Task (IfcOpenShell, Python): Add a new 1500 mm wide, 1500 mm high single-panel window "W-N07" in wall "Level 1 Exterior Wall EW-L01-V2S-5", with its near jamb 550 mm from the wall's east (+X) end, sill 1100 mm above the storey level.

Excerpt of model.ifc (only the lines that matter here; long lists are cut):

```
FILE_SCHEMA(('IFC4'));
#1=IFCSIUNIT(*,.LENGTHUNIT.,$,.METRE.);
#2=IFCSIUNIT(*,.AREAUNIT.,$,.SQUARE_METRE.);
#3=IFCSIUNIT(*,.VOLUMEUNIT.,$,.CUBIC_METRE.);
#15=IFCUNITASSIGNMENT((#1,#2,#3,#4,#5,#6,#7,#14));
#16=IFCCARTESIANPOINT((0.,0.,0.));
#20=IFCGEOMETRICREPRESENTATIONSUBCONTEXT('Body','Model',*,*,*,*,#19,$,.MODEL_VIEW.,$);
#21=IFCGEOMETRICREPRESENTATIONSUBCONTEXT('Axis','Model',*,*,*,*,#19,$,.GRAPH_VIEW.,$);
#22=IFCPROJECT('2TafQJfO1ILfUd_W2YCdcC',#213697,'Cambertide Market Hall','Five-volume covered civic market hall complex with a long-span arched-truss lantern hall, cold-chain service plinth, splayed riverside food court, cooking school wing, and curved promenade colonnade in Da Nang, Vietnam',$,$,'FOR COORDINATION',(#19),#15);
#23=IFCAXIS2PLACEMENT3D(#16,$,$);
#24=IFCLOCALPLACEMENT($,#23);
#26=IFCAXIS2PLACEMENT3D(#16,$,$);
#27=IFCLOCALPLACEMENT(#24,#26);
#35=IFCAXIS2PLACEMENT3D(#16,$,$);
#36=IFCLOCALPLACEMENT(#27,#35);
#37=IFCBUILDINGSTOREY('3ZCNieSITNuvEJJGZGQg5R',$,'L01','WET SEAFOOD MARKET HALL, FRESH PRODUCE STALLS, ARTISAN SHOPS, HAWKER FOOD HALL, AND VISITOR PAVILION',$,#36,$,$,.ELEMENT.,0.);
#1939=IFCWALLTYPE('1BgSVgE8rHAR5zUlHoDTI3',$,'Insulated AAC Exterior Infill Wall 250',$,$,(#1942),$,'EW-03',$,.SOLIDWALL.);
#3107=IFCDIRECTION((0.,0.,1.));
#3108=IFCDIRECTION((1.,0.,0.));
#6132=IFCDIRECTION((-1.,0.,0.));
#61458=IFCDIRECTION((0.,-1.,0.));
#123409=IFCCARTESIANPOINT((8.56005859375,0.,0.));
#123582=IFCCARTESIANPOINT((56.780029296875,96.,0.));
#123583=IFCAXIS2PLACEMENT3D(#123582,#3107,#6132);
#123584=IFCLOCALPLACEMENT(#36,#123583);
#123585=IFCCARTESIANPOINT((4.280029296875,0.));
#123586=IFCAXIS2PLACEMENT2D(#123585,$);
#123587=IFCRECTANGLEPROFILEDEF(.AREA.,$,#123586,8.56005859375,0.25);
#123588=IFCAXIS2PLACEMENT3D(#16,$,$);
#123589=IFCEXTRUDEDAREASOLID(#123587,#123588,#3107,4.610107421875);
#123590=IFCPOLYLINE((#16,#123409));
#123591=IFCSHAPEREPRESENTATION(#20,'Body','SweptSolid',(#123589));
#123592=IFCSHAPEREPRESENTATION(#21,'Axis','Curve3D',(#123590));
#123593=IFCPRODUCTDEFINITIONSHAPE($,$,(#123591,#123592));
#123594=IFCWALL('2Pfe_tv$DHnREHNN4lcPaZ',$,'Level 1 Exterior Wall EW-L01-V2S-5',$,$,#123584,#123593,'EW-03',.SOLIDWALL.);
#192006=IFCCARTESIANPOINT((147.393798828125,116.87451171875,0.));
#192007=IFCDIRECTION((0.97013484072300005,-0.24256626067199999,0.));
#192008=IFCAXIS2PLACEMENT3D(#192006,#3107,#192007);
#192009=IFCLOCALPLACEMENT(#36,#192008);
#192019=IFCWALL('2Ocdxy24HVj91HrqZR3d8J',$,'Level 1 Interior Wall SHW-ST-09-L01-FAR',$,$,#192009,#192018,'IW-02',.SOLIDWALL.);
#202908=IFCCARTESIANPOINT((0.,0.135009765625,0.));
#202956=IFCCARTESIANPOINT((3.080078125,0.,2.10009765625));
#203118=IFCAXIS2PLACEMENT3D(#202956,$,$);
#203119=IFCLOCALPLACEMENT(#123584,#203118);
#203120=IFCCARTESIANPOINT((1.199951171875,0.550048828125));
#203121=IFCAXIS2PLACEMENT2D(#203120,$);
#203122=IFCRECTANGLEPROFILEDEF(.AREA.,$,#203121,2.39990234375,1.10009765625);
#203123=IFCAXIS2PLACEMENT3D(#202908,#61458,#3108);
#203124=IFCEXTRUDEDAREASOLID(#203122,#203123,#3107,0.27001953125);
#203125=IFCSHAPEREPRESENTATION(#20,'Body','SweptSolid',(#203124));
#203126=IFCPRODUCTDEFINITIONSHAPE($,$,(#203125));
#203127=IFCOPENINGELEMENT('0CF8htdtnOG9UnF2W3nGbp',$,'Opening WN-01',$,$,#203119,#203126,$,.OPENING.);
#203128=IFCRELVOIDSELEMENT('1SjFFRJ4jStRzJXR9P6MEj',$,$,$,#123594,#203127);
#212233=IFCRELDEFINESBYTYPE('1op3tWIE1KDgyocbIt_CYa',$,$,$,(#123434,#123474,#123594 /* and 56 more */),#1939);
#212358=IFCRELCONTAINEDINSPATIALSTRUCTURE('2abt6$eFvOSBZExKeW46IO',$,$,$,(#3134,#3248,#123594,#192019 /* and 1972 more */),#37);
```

```python
import numpy as np
import ifcopenshell
import ifcopenshell.api.feature
import ifcopenshell.api.geometry
import ifcopenshell.api.root
import ifcopenshell.api.spatial
import ifcopenshell.geom
import ifcopenshell.util.element
import ifcopenshell.util.placement
import ifcopenshell.util.representation
import ifcopenshell.util.shape
import ifcopenshell.util.unit

model = ifcopenshell.open("model.ifc")
unit_scale = ifcopenshell.util.unit.calculate_unit_scale(model)
settings = ifcopenshell.geom.settings()


def volume(element):
    """Net volume in cubic metres, openings subtracted."""
    shape = ifcopenshell.geom.create_shape(settings, element)
    return ifcopenshell.util.shape.get_volume(shape.geometry)


wall = model.by_id(123594)
storey = ifcopenshell.util.element.get_container(wall, ifc_class="IfcBuildingStorey")
context = ifcopenshell.util.representation.get_context(model, "Model", "Body", "MODEL_VIEW")
before = volume(wall)

width, height, from_end, sill = 1.5, 1.5, 0.55, 1.1  # metres

# The wall runs along its own X axis, and the end named is its -X end.
wall_shape = ifcopenshell.geom.create_shape(settings, wall)
x, y, z = ifcopenshell.util.shape.get_vertices(wall_shape.geometry).T
start = x.min() + from_end
face, thickness = float(y.min()), float(y.max() - y.min())
wall_matrix = ifcopenshell.util.placement.get_local_placement(wall.ObjectPlacement)
level = ifcopenshell.util.placement.get_local_placement(storey.ObjectPlacement)[2, 3]


def in_wall(x, y):
    """Placement at x, y metres in the wall's axes, at sill height."""
    matrix = wall_matrix.copy()
    matrix[:, 3] = wall_matrix @ np.array([x / unit_scale, y / unit_scale, 0.0, 1.0])
    matrix[2, 3] = level + sill / unit_scale
    return matrix


# Opening: a box that overshoots both wall faces by 50 mm.
opening = ifcopenshell.api.root.create_entity(model, ifc_class="IfcOpeningElement", predefined_type="OPENING")
box = ifcopenshell.api.geometry.add_wall_representation(
    model, context=context, length=width, height=height, thickness=thickness + 0.1
)
ifcopenshell.api.geometry.assign_representation(model, product=opening, representation=box)
ifcopenshell.api.geometry.edit_object_placement(model, product=opening, matrix=in_wall(start, face - 0.05), is_si=False)
ifcopenshell.api.feature.add_feature(model, feature=opening, element=wall)

window = ifcopenshell.api.root.create_entity(model, ifc_class="IfcWindow", name="W-N07", predefined_type="WINDOW")
window.OverallWidth, window.OverallHeight = width / unit_scale, height / unit_scale
window.PartitioningType = "SINGLE_PANEL"
body = ifcopenshell.api.geometry.add_window_representation(
    model,
    context=context,
    overall_width=window.OverallWidth,
    overall_height=window.OverallHeight,
    partition_type="SINGLE_PANEL",
)
ifcopenshell.api.geometry.assign_representation(model, product=window, representation=body)
ifcopenshell.api.spatial.assign_container(model, products=[window], relating_structure=storey)
ifcopenshell.api.feature.add_filling(model, opening=opening, element=window)

# Centre the window in the wall's thickness.
ifcopenshell.api.geometry.edit_object_placement(model, product=window, matrix=in_wall(start, face), is_si=False)
window_shape = ifcopenshell.geom.create_shape(settings, window)
depth = ifcopenshell.util.shape.get_vertices(window_shape.geometry)[:, 1]
offset = face + thickness / 2 - (depth.min() + depth.max()) / 2
ifcopenshell.api.geometry.edit_object_placement(model, product=window, matrix=in_wall(start, offset), is_si=False)

after = volume(wall)

print(f"wall volume {before:.3f} -> {after:.3f} m3")

model.write("model_rev.ifc")
```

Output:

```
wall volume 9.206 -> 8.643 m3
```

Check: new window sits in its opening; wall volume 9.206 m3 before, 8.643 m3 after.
